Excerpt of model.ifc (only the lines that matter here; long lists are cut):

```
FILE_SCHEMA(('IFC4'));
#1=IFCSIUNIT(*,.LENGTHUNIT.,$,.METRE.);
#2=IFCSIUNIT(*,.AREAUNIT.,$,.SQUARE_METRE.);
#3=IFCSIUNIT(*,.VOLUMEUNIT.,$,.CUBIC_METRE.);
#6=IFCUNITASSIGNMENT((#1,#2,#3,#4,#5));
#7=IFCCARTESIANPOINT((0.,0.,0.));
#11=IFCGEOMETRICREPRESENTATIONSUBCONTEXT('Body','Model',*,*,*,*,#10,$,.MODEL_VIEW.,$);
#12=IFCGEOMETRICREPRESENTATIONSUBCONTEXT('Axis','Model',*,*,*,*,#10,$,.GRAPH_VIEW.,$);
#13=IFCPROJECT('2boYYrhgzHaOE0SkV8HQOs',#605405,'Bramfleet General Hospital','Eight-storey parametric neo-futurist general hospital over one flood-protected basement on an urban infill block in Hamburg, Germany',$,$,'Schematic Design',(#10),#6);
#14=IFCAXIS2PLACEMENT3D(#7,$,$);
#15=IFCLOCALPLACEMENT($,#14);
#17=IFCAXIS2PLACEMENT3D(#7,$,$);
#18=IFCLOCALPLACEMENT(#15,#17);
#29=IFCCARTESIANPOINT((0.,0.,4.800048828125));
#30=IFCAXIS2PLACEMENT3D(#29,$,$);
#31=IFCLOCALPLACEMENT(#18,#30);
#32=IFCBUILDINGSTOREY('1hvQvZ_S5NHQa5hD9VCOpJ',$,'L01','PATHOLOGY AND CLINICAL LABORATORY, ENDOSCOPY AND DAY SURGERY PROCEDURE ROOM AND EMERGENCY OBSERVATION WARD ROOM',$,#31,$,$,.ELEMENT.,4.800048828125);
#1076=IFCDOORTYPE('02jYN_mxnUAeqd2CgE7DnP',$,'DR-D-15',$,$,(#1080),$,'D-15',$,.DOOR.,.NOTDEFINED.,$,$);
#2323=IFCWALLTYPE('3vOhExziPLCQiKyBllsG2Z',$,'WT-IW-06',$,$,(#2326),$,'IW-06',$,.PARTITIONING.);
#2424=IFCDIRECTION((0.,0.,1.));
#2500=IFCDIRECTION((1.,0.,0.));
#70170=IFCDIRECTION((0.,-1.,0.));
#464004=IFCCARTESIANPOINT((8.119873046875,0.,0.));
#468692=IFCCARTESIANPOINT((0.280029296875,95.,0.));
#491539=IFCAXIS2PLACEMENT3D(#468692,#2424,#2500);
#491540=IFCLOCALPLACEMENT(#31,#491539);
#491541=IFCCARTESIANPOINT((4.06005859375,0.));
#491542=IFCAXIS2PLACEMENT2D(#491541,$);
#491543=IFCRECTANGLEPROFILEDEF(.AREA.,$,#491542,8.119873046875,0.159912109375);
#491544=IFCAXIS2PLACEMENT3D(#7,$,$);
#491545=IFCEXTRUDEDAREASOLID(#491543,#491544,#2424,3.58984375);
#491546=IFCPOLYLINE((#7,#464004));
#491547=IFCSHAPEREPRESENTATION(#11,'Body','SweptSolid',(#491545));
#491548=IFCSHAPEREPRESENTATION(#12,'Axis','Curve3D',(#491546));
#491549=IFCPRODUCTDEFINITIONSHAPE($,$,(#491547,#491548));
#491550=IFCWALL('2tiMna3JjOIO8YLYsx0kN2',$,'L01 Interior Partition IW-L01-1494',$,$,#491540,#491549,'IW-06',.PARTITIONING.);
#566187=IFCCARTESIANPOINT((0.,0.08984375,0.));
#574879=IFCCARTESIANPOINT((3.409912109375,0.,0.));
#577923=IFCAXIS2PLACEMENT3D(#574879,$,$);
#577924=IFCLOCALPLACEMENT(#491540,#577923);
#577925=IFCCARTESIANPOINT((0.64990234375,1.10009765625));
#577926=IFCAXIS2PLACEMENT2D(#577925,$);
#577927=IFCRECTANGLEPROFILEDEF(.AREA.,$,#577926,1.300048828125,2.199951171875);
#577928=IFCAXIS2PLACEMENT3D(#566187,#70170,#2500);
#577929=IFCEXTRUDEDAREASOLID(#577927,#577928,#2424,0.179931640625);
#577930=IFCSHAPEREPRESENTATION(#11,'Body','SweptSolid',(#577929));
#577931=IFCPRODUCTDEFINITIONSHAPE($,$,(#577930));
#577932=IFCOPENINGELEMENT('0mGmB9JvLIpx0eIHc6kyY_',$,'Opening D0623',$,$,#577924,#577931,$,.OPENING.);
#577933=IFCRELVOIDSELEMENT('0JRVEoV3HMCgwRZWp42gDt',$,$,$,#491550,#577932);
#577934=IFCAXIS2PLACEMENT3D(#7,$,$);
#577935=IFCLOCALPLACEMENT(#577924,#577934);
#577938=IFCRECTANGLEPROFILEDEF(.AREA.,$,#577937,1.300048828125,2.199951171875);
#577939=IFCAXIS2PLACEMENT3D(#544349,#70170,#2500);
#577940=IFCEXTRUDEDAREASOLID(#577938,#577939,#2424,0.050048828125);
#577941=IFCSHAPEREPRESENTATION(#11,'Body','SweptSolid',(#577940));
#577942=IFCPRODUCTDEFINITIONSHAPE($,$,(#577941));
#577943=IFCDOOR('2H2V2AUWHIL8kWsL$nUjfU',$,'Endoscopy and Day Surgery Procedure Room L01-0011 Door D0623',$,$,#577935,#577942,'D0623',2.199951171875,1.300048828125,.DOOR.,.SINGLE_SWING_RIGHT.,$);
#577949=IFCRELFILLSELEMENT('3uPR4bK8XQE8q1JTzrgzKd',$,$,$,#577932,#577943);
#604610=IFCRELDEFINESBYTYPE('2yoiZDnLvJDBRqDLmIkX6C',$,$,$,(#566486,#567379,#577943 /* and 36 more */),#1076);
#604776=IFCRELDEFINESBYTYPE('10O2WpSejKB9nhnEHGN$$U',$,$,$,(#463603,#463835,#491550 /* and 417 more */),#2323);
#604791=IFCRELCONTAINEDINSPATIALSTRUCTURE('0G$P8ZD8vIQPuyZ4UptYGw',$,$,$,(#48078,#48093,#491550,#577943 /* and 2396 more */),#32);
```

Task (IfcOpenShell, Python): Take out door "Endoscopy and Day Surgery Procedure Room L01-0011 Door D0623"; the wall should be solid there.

```python
import ifcopenshell
import ifcopenshell.api.feature
import ifcopenshell.api.root
import ifcopenshell.geom
import ifcopenshell.util.shape

model = ifcopenshell.open("model.ifc")
settings = ifcopenshell.geom.settings()


def volume(element):
    """Net volume in cubic metres, openings subtracted."""
    shape = ifcopenshell.geom.create_shape(settings, element)
    return ifcopenshell.util.shape.get_volume(shape.geometry)


door = model.by_id(577943)
opening = door.FillsVoids[0].RelatingOpeningElement
wall = opening.VoidsElements[0].RelatingBuildingElement
before = volume(wall)

ifcopenshell.api.root.remove_product(model, product=door)
ifcopenshell.api.feature.remove_feature(model, feature=opening)

after = volume(wall)

print(f"wall volume {before:.3f} -> {after:.3f} m3")

model.write("model_edited.ifc")
```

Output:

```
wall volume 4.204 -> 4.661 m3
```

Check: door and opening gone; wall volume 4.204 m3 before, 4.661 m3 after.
